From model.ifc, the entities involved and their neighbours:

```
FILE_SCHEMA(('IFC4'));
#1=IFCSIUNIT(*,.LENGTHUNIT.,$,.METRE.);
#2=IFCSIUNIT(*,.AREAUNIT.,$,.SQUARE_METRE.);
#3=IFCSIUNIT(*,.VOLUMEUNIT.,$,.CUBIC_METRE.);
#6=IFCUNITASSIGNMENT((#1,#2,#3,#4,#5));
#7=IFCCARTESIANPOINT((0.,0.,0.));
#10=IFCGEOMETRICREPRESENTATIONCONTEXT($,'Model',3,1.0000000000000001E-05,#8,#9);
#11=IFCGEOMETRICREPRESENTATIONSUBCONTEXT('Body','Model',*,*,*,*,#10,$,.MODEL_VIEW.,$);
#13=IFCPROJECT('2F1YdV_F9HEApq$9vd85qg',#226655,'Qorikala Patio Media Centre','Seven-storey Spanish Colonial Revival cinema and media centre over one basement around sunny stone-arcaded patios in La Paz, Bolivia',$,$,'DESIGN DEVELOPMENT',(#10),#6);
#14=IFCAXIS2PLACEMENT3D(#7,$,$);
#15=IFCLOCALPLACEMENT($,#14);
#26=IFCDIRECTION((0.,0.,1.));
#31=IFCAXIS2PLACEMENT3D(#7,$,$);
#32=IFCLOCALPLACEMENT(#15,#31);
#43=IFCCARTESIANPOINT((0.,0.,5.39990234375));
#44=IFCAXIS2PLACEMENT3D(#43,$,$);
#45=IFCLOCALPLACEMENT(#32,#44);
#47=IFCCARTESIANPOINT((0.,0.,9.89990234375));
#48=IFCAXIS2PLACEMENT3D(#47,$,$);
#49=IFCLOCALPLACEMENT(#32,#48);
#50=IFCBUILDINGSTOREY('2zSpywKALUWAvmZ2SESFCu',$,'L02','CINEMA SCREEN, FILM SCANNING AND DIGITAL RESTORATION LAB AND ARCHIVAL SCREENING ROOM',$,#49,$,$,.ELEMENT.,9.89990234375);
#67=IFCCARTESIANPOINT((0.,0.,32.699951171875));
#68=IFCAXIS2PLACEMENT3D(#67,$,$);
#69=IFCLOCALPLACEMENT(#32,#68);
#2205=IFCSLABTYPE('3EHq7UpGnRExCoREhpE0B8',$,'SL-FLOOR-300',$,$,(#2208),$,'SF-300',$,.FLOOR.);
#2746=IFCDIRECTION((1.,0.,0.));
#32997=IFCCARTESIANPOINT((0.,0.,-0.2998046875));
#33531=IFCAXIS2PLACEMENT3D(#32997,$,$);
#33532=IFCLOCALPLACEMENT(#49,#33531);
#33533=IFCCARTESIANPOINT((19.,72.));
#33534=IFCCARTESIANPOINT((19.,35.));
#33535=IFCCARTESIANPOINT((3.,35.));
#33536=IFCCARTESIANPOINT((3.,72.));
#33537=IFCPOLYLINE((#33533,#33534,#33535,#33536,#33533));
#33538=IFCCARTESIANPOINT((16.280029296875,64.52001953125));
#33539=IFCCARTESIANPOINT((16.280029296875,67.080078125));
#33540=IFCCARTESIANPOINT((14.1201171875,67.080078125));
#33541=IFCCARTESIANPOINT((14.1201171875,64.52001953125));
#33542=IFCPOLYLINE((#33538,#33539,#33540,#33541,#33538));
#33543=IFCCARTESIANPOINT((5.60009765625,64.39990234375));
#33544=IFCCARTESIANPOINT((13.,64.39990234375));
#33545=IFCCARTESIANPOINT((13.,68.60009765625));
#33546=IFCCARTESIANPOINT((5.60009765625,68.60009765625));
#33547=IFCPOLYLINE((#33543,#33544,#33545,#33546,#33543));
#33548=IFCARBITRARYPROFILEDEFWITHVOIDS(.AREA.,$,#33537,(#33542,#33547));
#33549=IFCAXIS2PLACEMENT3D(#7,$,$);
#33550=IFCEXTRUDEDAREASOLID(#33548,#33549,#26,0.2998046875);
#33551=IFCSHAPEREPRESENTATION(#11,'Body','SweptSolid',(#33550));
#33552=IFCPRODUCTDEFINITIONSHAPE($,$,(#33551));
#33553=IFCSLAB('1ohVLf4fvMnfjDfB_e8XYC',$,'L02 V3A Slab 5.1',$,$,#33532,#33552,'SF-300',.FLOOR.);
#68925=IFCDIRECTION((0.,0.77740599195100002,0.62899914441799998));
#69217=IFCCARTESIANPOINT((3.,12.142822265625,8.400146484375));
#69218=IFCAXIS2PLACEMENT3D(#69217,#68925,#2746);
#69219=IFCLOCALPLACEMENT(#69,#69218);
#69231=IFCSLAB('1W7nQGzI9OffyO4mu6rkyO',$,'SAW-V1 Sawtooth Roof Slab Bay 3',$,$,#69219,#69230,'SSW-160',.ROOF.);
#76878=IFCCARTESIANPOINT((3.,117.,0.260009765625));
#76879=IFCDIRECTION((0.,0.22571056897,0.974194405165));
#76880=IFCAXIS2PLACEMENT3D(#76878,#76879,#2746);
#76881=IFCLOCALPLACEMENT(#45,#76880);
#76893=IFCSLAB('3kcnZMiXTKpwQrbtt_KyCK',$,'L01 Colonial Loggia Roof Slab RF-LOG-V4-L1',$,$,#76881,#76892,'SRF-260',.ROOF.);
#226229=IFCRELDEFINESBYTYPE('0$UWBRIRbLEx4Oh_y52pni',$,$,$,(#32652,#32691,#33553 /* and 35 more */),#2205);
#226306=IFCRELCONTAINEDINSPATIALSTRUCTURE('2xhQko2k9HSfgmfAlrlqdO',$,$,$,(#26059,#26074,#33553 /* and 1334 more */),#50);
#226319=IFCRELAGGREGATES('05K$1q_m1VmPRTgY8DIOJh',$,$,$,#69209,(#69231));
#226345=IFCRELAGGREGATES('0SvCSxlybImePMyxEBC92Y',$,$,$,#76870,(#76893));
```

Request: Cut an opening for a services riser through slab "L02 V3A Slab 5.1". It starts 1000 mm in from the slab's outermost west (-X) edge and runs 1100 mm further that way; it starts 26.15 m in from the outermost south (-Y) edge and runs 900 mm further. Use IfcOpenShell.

```python
import numpy as np
import ifcopenshell
import ifcopenshell.api.feature
import ifcopenshell.api.geometry
import ifcopenshell.api.root
import ifcopenshell.geom
import ifcopenshell.util.placement
import ifcopenshell.util.representation
import ifcopenshell.util.shape
import ifcopenshell.util.unit

model = ifcopenshell.open("model.ifc")
unit_scale = ifcopenshell.util.unit.calculate_unit_scale(model)
settings = ifcopenshell.geom.settings()


def volume(element):
    """Net volume in cubic metres, openings subtracted."""
    shape = ifcopenshell.geom.create_shape(settings, element)
    return ifcopenshell.util.shape.get_volume(shape.geometry)


slab = model.by_guid("1ohVLf4fvMnfjDfB_e8XYC")
before = volume(slab)

# Extent in the slab's own axes, in metres. The edges named are its -X and -Y sides.
slab_shape = ifcopenshell.geom.create_shape(settings, slab)
vertices = ifcopenshell.util.shape.get_vertices(slab_shape.geometry)
x_min, y_min, bottom = vertices.min(axis=0)
top = vertices[:, 2].max()

opening = ifcopenshell.api.root.create_entity(model, ifc_class="IfcOpeningElement", name="Services riser opening", predefined_type="OPENING")
context = ifcopenshell.util.representation.get_context(model, "Model", "Body", "MODEL_VIEW")
width, depth = 1.1, 0.9
outline = [(0.0, 0.0), (width, 0.0), (width, depth), (0.0, depth), (0.0, 0.0)]
# Overshoot both faces by 50 mm so the cut is clean.
shape = ifcopenshell.api.geometry.add_slab_representation(
    model, context=context, depth=top - bottom + 0.1, polyline=outline
)
ifcopenshell.api.geometry.assign_representation(model, product=opening, representation=shape)

matrix = ifcopenshell.util.placement.get_local_placement(slab.ObjectPlacement)
matrix[:, 3] = matrix @ np.append(np.array([x_min + 1, y_min + 26.15, bottom - 0.05]) / unit_scale, 1.0)
ifcopenshell.api.geometry.edit_object_placement(model, product=opening, matrix=matrix, is_si=False)
ifcopenshell.api.feature.add_feature(model, feature=opening, element=slab)

after = volume(slab)

print(f"slab volume {before:.3f} -> {after:.3f} m3")

model.write("model_v2.ifc")
```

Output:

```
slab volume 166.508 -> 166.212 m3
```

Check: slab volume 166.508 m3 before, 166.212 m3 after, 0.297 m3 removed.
